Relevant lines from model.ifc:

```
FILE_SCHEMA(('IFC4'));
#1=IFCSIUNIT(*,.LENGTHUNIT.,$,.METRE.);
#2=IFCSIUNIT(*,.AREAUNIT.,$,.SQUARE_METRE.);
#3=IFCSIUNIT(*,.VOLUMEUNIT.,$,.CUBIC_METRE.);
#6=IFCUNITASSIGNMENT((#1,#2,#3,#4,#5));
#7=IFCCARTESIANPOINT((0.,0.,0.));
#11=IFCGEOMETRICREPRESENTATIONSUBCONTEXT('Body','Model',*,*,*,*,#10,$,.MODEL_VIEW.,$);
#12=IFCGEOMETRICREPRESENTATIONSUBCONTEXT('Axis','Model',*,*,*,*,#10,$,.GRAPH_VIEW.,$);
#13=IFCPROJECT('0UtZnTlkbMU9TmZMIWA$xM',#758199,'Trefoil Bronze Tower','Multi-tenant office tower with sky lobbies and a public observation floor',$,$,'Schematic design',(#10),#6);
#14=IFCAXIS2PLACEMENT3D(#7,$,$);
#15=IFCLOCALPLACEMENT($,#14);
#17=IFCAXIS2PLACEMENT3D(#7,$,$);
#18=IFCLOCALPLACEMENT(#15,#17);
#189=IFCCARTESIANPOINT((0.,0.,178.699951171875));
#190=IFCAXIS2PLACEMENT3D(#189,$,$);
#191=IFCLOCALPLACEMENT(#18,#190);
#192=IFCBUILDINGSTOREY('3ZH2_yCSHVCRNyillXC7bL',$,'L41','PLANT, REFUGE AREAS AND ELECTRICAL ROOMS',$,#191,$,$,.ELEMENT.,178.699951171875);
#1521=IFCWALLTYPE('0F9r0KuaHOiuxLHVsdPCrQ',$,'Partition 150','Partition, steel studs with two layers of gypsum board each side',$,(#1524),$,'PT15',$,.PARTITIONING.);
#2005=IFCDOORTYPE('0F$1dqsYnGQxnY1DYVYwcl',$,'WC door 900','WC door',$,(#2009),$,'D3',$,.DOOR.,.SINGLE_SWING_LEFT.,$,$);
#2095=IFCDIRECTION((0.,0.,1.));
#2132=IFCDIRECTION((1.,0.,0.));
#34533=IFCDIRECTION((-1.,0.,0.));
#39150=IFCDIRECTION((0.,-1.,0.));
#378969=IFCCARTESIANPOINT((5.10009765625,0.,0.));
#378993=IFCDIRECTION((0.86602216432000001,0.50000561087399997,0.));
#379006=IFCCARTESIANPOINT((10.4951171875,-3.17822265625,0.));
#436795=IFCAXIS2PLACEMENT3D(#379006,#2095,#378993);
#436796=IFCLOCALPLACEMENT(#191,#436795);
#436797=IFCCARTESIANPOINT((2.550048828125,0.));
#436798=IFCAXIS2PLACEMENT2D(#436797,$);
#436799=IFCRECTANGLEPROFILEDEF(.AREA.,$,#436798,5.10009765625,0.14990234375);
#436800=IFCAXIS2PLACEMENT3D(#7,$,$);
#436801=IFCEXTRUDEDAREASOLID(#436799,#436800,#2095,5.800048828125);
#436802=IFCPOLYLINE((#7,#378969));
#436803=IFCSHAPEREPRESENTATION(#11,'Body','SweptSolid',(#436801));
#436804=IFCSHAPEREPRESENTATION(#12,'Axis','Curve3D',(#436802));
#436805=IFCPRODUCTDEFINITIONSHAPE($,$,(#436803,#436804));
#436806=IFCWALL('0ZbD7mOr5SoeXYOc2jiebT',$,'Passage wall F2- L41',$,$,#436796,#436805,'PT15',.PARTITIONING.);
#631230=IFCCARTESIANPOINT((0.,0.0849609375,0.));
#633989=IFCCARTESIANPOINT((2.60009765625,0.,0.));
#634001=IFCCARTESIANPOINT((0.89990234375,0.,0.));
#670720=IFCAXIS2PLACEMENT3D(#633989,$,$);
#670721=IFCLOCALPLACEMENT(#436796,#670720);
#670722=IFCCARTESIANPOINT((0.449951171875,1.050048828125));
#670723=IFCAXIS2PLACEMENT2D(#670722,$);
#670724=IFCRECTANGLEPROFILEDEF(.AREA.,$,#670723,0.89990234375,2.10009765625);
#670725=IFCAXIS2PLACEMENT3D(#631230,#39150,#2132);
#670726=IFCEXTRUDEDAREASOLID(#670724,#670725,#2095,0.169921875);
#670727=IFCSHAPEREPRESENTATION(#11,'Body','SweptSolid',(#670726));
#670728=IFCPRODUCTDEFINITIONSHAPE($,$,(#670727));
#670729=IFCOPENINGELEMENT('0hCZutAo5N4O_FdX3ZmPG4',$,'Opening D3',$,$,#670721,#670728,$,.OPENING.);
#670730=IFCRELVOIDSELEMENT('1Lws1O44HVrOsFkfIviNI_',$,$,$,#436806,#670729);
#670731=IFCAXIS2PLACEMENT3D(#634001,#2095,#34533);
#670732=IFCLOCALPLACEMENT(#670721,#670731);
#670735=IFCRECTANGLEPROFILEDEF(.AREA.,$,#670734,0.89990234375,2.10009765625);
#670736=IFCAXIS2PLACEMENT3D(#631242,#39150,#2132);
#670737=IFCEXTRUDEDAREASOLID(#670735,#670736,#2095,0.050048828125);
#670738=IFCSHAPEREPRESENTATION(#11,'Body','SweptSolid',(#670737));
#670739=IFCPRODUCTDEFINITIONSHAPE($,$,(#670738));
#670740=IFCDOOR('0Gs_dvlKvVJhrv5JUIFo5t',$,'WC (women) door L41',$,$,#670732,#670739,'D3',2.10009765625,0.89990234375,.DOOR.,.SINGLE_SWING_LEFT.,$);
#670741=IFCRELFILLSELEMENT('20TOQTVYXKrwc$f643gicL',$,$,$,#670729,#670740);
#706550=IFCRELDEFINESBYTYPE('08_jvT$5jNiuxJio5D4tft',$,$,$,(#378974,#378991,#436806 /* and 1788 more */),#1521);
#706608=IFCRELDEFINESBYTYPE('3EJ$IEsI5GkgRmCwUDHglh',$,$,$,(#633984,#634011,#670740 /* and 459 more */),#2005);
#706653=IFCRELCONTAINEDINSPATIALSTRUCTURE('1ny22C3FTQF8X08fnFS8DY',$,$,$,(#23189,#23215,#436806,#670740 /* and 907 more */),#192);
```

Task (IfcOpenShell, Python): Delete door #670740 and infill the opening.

```python
import ifcopenshell
import ifcopenshell.api.feature
import ifcopenshell.api.root
import ifcopenshell.geom
import ifcopenshell.util.shape

model = ifcopenshell.open("model.ifc")
settings = ifcopenshell.geom.settings()


def volume(element):
    """Net volume in cubic metres, openings subtracted."""
    shape = ifcopenshell.geom.create_shape(settings, element)
    return ifcopenshell.util.shape.get_volume(shape.geometry)


door = model.by_id(670740)
opening = door.FillsVoids[0].RelatingOpeningElement
wall = opening.VoidsElements[0].RelatingBuildingElement
before = volume(wall)

ifcopenshell.api.root.remove_product(model, product=door)
ifcopenshell.api.feature.remove_feature(model, feature=opening)

after = volume(wall)

print(f"wall volume {before:.3f} -> {after:.3f} m3")

model.write("model_v2.ifc")
```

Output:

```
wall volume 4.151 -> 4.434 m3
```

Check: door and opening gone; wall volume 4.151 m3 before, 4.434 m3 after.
